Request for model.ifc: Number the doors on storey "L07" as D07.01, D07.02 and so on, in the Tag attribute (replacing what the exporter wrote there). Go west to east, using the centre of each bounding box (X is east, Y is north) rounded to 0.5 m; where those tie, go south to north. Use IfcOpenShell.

First a look at what the model holds.

```python
import ifcopenshell
import ifcopenshell.util.element
import ifcopenshell.util.placement

model = ifcopenshell.open("model.ifc")
print(model.schema)
storey = next(s for s in model.by_type("IfcBuildingStorey") if s.Name == "L07")
doors = [e for e in ifcopenshell.util.element.get_decomposition(storey) if e.is_a("IfcDoor")]
for e in sorted(doors, key=lambda e: e.id()):
    origin = ifcopenshell.util.placement.get_local_placement(e.ObjectPlacement)[:3, 3]
    print(e.id(), e.Tag, e.Name, origin.round(2) + 0.0, sep=" | ")
```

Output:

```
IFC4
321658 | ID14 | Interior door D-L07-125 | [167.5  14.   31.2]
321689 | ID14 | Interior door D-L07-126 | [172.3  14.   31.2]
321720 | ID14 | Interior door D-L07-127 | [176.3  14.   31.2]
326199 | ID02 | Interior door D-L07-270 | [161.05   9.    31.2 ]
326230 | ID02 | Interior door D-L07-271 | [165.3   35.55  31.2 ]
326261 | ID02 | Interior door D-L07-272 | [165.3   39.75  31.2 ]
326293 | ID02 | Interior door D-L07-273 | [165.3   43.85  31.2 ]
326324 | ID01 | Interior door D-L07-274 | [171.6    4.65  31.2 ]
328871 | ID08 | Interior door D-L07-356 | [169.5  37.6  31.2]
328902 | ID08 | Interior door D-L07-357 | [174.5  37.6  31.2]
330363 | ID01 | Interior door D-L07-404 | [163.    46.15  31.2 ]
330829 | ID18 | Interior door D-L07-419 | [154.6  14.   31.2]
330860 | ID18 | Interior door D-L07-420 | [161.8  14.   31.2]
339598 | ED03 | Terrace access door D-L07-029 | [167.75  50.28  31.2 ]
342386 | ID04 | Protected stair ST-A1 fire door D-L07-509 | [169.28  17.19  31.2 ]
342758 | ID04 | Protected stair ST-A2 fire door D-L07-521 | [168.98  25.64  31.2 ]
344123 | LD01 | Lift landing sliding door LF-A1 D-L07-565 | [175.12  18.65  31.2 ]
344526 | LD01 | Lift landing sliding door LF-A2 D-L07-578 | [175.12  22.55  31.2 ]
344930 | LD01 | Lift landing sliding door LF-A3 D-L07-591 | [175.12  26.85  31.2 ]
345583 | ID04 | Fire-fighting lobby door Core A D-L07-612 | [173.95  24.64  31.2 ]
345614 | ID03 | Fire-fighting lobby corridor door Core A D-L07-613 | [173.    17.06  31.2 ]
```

```python
import ifcopenshell
import ifcopenshell.geom
import ifcopenshell.util.element
import ifcopenshell.util.shape

model = ifcopenshell.open("model.ifc")
settings = ifcopenshell.geom.settings()
settings.set("use-world-coords", True)


def centre(element):
    shape = ifcopenshell.geom.create_shape(settings, element)
    return ifcopenshell.util.shape.get_bbox_centroid(shape.geometry)


storey = next(s for s in model.by_type("IfcBuildingStorey") if s.Name == "L07")
doors = [e for e in ifcopenshell.util.element.get_decomposition(storey) if e.is_a("IfcDoor")]

# Insertion points can sit at a corner or the storey origin, so sort by the geometry (in metres).
centres = {e: centre(e) for e in doors}
doors.sort(key=lambda e: (round(centres[e][0] / 0.5), centres[e][1]))

for i, e in enumerate(doors, start=1):
    number = f"D07.{i:02d}"
    e.Tag = number
    print(e.id(), number)

model.write("model_v2.ifc")
```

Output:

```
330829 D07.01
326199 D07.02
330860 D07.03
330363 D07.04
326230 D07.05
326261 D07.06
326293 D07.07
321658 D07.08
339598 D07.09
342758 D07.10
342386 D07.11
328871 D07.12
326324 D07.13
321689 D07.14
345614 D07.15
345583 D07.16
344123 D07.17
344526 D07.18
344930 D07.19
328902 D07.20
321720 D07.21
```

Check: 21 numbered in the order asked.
